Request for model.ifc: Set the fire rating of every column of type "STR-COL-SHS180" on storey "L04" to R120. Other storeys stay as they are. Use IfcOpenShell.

First a look at what the model holds.

```python
import ifcopenshell
import ifcopenshell.util.element

model = ifcopenshell.open("model.ifc")
print(model.schema)
storey = next(s for s in model.by_type("IfcBuildingStorey") if s.Name == "L04")
columns = [e for e in ifcopenshell.util.element.get_decomposition(storey) if e.is_a("IfcColumn")]
seen = {}
for e in columns:
    element_type = ifcopenshell.util.element.get_type(e)
    key = (element_type.Name if element_type != e and element_type else None, ifcopenshell.util.element.get_pset(e, "Pset_ColumnCommon", "FireRating"))
    seen[key] = seen.get(key, 0) + 1
for (name, value), count in sorted(seen.items(), key=str):
    print(count, "x", name, "|", value)
```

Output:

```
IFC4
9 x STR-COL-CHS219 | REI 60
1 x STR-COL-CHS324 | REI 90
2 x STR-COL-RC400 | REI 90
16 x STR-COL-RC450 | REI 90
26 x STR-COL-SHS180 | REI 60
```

```python
import ifcopenshell
import ifcopenshell.api.pset
import ifcopenshell.util.element

model = ifcopenshell.open("model.ifc")

storey = next(s for s in model.by_type("IfcBuildingStorey") if s.Name == "L04")
columns = [e for e in ifcopenshell.util.element.get_decomposition(storey) if e.is_a("IfcColumn")]

count = 0
for e in columns:
    element_type = ifcopenshell.util.element.get_type(e)
    if element_type in (None, e) or element_type.Name != "STR-COL-SHS180":
        continue
    # add_pset returns the element's existing set when there is one.
    pset = ifcopenshell.api.pset.add_pset(model, product=e, name="Pset_ColumnCommon")
    ifcopenshell.api.pset.edit_pset(model, pset=pset, properties={"FireRating": "R120"})
    count += 1

print(count, "columns updated")

model.write("model_edited.ifc")
```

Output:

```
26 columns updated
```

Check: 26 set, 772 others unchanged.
